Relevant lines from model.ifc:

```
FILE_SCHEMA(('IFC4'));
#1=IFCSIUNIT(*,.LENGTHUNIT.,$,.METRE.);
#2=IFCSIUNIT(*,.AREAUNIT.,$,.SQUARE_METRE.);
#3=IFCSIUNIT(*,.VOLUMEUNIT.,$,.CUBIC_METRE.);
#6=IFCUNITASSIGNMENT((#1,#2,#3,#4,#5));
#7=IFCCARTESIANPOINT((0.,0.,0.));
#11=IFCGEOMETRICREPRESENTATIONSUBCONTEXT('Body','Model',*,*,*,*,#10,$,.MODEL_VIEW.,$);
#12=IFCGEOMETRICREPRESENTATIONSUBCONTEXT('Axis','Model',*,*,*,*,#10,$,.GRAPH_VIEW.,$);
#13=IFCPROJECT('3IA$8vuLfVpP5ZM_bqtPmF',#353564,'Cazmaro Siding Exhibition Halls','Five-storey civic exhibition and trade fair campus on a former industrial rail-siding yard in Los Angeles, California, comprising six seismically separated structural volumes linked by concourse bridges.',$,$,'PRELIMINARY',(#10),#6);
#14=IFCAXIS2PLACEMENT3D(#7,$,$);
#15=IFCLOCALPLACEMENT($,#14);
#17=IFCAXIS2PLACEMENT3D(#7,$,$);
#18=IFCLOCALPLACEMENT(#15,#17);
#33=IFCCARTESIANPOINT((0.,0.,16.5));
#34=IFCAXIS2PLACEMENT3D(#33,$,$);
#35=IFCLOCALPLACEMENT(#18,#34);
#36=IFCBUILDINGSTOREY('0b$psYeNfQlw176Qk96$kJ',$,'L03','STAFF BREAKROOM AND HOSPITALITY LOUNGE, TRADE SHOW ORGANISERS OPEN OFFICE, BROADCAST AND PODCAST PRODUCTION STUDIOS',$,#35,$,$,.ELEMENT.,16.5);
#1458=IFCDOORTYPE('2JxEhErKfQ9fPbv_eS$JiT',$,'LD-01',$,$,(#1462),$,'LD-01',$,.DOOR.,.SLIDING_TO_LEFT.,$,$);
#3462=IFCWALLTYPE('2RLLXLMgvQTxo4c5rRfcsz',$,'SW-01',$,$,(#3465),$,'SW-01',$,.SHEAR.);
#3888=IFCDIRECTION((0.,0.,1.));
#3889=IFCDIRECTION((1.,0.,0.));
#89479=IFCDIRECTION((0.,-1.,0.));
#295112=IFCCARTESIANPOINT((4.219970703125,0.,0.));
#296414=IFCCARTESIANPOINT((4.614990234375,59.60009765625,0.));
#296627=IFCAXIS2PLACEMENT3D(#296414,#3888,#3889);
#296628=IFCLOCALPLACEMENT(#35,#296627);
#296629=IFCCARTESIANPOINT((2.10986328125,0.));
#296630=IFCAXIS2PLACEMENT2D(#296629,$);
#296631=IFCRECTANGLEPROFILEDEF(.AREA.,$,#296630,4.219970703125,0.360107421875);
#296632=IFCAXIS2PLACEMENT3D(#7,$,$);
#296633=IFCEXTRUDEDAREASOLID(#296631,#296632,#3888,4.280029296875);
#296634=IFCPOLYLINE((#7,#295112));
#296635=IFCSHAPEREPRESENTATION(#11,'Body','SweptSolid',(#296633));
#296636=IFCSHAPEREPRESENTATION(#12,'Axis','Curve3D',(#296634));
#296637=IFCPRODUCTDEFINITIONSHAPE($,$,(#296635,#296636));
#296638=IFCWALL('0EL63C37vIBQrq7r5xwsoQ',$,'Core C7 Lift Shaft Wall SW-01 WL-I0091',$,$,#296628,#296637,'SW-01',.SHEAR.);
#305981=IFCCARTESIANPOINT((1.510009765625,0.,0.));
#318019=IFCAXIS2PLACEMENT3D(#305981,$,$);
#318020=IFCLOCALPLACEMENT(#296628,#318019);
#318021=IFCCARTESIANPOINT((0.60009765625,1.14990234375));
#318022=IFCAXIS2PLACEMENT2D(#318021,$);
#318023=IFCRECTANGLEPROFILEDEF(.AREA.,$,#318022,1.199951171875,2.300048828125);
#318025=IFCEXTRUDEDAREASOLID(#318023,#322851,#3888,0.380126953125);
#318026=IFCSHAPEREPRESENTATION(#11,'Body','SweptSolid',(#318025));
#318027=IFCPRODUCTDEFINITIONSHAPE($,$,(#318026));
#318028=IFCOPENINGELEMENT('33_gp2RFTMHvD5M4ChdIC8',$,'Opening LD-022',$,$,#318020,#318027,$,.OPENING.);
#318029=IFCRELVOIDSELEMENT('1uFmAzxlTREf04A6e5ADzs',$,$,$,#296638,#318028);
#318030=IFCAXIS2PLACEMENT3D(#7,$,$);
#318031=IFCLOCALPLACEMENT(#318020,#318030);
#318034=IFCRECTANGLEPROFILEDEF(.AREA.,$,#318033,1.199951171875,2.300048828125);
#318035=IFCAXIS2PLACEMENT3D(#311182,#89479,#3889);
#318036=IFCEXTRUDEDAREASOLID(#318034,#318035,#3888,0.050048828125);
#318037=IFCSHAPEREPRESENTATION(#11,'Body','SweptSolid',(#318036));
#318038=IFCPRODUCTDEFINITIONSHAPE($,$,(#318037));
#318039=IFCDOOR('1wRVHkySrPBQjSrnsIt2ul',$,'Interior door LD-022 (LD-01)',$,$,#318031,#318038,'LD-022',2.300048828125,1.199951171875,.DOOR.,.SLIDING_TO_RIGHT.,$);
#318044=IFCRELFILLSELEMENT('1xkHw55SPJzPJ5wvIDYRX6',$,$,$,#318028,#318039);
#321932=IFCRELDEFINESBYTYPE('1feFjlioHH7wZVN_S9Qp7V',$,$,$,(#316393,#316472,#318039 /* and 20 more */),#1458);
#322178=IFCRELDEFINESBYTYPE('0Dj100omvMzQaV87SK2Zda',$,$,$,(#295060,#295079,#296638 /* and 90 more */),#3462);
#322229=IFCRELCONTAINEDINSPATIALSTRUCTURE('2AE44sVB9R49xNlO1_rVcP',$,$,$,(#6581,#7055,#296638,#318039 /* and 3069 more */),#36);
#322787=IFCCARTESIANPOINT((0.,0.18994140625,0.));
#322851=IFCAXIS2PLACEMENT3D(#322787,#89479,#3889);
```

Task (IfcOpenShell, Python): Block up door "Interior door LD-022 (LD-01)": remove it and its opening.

```python
import ifcopenshell
import ifcopenshell.api.feature
import ifcopenshell.api.root
import ifcopenshell.geom
import ifcopenshell.util.shape

model = ifcopenshell.open("model.ifc")
settings = ifcopenshell.geom.settings()


def volume(element):
    """Net volume in cubic metres, openings subtracted."""
    shape = ifcopenshell.geom.create_shape(settings, element)
    return ifcopenshell.util.shape.get_volume(shape.geometry)


door = model.by_guid("1wRVHkySrPBQjSrnsIt2ul")
opening = door.FillsVoids[0].RelatingOpeningElement
wall = opening.VoidsElements[0].RelatingBuildingElement
before = volume(wall)

ifcopenshell.api.root.remove_product(model, product=door)
ifcopenshell.api.feature.remove_feature(model, feature=opening)

after = volume(wall)

print(f"wall volume {before:.3f} -> {after:.3f} m3")

model.write("model_edited.ifc")
```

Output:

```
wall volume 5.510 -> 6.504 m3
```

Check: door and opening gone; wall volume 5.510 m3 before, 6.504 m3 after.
